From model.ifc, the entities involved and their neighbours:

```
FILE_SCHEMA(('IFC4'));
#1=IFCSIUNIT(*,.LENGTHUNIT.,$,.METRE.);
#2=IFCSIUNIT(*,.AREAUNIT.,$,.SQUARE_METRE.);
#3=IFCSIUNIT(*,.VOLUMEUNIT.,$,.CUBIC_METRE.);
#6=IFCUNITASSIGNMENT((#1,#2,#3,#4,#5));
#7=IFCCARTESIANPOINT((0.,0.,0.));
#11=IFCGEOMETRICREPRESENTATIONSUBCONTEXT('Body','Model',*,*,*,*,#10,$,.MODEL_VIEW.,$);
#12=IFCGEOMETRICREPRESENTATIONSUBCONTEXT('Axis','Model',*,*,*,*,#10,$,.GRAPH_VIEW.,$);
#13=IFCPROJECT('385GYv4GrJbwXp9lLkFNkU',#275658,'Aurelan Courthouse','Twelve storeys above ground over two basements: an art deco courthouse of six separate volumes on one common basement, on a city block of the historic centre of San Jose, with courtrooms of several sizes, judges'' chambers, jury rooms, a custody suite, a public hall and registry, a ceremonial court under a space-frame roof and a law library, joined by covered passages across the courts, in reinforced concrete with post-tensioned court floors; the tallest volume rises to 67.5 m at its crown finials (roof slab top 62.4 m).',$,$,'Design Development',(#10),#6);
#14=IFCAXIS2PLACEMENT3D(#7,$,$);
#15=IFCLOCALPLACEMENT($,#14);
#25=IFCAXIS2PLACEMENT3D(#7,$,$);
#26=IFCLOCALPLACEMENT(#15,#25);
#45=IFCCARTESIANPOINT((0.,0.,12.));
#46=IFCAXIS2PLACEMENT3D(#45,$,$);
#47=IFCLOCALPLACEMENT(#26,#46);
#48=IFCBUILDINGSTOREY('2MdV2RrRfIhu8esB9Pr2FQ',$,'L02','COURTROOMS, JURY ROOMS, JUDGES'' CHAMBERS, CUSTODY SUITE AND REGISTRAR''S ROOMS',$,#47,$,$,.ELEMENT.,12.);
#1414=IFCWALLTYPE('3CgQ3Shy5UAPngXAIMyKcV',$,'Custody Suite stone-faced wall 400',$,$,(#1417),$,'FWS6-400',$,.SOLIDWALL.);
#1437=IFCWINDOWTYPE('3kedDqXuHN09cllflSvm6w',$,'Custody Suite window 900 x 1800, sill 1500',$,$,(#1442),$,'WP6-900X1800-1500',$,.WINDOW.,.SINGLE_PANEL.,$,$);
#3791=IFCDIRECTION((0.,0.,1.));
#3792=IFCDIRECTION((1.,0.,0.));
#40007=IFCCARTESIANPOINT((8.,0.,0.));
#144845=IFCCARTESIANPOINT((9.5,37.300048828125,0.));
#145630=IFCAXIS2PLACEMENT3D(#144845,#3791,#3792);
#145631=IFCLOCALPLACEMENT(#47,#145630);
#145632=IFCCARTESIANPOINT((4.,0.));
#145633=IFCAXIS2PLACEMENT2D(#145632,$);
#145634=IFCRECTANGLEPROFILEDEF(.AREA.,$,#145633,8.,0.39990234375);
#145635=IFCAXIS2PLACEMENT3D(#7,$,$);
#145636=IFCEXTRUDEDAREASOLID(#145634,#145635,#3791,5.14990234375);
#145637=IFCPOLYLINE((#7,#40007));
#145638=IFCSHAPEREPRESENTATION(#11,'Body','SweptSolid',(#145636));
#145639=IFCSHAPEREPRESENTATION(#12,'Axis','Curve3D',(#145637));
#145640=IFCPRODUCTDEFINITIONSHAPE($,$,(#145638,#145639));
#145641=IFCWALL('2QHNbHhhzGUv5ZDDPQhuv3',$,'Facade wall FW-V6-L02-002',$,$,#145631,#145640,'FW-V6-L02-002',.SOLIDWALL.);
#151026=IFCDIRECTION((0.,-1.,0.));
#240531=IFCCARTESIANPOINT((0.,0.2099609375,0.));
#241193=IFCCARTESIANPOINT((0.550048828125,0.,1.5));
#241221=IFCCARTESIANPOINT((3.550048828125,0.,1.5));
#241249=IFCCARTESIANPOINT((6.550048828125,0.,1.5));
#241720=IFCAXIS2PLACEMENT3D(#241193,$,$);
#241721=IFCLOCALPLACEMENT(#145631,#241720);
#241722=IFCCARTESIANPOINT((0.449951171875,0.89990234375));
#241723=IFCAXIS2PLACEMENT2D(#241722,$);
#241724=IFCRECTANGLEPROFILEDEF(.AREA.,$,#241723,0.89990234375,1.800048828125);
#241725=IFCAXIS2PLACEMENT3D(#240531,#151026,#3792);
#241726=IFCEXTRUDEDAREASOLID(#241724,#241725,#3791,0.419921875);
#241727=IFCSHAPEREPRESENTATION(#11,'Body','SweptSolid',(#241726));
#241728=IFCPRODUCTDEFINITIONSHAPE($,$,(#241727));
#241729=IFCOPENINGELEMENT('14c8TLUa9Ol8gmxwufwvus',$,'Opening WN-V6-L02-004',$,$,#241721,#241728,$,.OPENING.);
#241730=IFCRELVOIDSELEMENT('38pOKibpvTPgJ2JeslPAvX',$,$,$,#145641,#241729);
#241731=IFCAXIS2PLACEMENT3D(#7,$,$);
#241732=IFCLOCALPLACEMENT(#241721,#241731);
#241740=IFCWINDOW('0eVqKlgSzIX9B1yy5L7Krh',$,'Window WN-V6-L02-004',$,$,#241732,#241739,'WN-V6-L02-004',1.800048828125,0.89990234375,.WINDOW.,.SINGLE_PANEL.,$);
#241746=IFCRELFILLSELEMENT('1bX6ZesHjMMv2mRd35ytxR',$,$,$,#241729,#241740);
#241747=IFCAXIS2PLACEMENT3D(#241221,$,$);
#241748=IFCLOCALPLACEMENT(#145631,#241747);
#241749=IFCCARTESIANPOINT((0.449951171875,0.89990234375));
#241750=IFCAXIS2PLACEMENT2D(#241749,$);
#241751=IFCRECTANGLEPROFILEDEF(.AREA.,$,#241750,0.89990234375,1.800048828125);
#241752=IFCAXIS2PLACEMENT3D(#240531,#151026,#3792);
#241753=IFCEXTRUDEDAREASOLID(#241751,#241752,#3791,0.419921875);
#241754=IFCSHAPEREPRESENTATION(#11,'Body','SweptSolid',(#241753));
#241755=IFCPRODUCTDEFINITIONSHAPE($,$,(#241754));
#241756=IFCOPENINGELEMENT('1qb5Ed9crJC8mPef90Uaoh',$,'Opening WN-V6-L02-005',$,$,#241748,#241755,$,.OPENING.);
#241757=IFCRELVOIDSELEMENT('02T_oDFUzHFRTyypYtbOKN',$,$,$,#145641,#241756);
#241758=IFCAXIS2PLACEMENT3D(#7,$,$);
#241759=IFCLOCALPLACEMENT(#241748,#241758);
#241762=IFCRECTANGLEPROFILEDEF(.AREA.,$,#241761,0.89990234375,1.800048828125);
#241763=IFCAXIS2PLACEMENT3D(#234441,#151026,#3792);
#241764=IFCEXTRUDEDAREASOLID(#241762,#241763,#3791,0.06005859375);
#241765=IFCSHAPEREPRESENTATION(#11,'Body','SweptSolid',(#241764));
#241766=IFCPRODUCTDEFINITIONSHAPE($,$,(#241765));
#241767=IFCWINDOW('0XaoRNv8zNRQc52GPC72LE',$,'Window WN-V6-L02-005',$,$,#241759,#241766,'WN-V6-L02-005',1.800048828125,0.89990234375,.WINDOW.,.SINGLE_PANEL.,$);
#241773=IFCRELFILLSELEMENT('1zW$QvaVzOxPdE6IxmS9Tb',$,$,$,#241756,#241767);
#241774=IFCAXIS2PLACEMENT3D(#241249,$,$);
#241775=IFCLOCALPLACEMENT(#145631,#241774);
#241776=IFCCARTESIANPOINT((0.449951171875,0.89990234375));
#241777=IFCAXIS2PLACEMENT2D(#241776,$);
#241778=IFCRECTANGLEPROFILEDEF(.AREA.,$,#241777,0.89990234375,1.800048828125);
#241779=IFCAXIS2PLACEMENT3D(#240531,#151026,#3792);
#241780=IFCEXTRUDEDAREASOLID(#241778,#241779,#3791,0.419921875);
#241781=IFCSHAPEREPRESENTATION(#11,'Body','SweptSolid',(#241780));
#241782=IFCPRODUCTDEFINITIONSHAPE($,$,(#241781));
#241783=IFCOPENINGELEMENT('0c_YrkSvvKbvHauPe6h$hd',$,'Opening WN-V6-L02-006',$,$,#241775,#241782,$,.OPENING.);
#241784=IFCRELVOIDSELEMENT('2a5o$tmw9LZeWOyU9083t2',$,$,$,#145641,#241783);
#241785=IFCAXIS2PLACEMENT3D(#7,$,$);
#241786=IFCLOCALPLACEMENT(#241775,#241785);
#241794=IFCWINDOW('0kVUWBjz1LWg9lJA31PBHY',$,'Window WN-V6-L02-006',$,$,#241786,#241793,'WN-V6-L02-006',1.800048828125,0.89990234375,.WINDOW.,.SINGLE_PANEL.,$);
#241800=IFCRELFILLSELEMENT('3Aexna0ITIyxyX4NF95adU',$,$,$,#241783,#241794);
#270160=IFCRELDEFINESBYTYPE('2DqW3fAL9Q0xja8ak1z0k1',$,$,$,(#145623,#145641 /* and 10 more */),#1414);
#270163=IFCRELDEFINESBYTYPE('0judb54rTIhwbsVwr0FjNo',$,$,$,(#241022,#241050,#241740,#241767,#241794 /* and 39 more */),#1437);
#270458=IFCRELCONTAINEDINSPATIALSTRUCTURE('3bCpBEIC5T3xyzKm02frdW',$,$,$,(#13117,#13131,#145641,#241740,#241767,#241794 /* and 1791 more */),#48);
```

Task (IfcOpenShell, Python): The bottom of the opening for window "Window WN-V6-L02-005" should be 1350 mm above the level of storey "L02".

```python
import numpy as np
import ifcopenshell
import ifcopenshell.api.geometry
import ifcopenshell.geom
import ifcopenshell.util.element
import ifcopenshell.util.placement
import ifcopenshell.util.shape
import ifcopenshell.util.unit

model = ifcopenshell.open("model.ifc")
unit_scale = ifcopenshell.util.unit.calculate_unit_scale(model)

window = model.by_guid("0XaoRNv8zNRQc52GPC72LE")
opening = window.FillsVoids[0].RelatingOpeningElement
storey = ifcopenshell.util.element.get_container(window, ifc_class="IfcBuildingStorey")
level = ifcopenshell.util.placement.get_local_placement(storey.ObjectPlacement)[2, 3]

# The opening's origin need not be at the sill, so measure its lowest point.
shape = ifcopenshell.geom.create_shape(ifcopenshell.geom.settings(), opening)
bottom = ifcopenshell.util.shape.get_shape_bottom_elevation(shape, shape.geometry) / unit_scale
dz = level + 1.35 - bottom

shift = np.array([0.0, 0.0, dz])
# The window is placed relative to its opening, so it follows when the opening moves.
matrix = ifcopenshell.util.placement.get_local_placement(opening.ObjectPlacement)
matrix[:3, 3] += shift
ifcopenshell.api.geometry.edit_object_placement(
    model, product=opening, matrix=matrix, is_si=False, should_transform_children=True
)

print(f"moved by {dz * unit_scale:+.3f} m")

model.write("model-out.ifc")
```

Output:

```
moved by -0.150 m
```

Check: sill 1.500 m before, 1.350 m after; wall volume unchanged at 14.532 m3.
